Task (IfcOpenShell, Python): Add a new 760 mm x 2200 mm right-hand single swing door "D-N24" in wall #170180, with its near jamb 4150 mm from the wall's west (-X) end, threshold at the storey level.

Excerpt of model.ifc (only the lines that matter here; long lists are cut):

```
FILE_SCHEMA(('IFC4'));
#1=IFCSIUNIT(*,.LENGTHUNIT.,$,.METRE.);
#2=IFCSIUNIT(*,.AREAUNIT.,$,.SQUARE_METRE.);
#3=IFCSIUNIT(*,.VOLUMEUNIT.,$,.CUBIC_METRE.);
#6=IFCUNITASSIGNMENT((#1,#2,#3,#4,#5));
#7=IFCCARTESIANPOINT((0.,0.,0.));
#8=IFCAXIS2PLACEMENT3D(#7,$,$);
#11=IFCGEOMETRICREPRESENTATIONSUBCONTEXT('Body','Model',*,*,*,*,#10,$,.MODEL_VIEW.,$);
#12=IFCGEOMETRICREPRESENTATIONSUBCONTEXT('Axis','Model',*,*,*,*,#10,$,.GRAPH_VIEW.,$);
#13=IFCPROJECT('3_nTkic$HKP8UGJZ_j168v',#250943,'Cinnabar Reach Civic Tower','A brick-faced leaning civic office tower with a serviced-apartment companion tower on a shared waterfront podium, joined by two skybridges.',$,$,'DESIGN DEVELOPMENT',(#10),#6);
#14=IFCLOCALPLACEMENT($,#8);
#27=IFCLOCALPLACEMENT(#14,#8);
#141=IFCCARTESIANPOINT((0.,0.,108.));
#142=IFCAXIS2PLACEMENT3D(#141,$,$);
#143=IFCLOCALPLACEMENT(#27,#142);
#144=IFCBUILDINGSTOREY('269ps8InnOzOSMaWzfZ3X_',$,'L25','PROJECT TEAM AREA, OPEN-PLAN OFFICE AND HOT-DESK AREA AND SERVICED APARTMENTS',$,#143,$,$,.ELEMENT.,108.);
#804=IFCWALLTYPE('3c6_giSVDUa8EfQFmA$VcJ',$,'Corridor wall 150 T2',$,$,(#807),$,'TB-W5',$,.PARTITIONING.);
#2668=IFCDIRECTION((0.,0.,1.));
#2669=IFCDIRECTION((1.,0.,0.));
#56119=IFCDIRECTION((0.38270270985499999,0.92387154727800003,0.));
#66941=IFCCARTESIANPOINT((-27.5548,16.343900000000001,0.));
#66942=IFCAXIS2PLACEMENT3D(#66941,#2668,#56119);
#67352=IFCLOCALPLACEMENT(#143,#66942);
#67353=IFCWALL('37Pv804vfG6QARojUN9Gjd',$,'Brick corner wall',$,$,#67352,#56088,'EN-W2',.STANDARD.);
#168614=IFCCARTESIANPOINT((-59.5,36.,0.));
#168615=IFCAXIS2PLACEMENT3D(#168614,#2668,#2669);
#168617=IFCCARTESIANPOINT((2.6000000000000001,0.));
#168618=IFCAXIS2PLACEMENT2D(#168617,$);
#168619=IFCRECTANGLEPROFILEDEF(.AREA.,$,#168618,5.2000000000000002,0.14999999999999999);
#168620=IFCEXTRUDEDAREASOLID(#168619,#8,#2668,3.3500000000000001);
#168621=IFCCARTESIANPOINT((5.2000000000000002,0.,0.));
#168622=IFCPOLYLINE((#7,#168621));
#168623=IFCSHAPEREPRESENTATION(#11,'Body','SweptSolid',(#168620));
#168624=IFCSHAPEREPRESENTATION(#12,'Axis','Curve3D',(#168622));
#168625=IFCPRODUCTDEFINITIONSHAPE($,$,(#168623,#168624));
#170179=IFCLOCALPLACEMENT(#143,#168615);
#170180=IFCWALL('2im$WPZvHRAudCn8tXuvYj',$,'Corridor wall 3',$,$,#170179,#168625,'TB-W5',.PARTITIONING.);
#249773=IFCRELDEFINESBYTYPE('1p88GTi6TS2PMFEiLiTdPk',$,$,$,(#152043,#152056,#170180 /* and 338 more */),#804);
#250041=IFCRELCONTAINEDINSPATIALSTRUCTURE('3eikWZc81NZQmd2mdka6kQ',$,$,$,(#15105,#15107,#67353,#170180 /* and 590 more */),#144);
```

```python
import numpy as np
import ifcopenshell
import ifcopenshell.api.feature
import ifcopenshell.api.geometry
import ifcopenshell.api.root
import ifcopenshell.api.spatial
import ifcopenshell.geom
import ifcopenshell.util.element
import ifcopenshell.util.placement
import ifcopenshell.util.representation
import ifcopenshell.util.shape
import ifcopenshell.util.unit

model = ifcopenshell.open("model.ifc")
unit_scale = ifcopenshell.util.unit.calculate_unit_scale(model)
settings = ifcopenshell.geom.settings()


def volume(element):
    """Net volume in cubic metres, openings subtracted."""
    shape = ifcopenshell.geom.create_shape(settings, element)
    return ifcopenshell.util.shape.get_volume(shape.geometry)


wall = model.by_guid("2im$WPZvHRAudCn8tXuvYj")
storey = ifcopenshell.util.element.get_container(wall, ifc_class="IfcBuildingStorey")
context = ifcopenshell.util.representation.get_context(model, "Model", "Body", "MODEL_VIEW")
before = volume(wall)

width, height, from_end, sill = 0.76, 2.2, 4.15, 0.0  # metres

# The wall runs along its own X axis, and the end named is its -X end.
wall_shape = ifcopenshell.geom.create_shape(settings, wall)
x, y, z = ifcopenshell.util.shape.get_vertices(wall_shape.geometry).T
start = x.min() + from_end
face, thickness = float(y.min()), float(y.max() - y.min())
wall_matrix = ifcopenshell.util.placement.get_local_placement(wall.ObjectPlacement)
level = ifcopenshell.util.placement.get_local_placement(storey.ObjectPlacement)[2, 3]


def in_wall(x, y):
    """Placement at x, y metres in the wall's axes, at sill height."""
    matrix = wall_matrix.copy()
    matrix[:, 3] = wall_matrix @ np.array([x / unit_scale, y / unit_scale, 0.0, 1.0])
    matrix[2, 3] = level + sill / unit_scale
    return matrix


# Opening: a box that overshoots both wall faces by 50 mm.
opening = ifcopenshell.api.root.create_entity(model, ifc_class="IfcOpeningElement", predefined_type="OPENING")
box = ifcopenshell.api.geometry.add_wall_representation(
    model, context=context, length=width, height=height, thickness=thickness + 0.1
)
ifcopenshell.api.geometry.assign_representation(model, product=opening, representation=box)
ifcopenshell.api.geometry.edit_object_placement(model, product=opening, matrix=in_wall(start, face - 0.05), is_si=False)
ifcopenshell.api.feature.add_feature(model, feature=opening, element=wall)

door = ifcopenshell.api.root.create_entity(model, ifc_class="IfcDoor", name="D-N24", predefined_type="DOOR")
door.OverallWidth, door.OverallHeight = width / unit_scale, height / unit_scale
door.OperationType = "SINGLE_SWING_RIGHT"
body = ifcopenshell.api.geometry.add_door_representation(
    model,
    context=context,
    overall_width=door.OverallWidth,
    overall_height=door.OverallHeight,
    operation_type="SINGLE_SWING_RIGHT",
    lining_properties={"LiningDepth": thickness / unit_scale, "ThresholdDepth": thickness / unit_scale},
)
ifcopenshell.api.geometry.assign_representation(model, product=door, representation=body)
ifcopenshell.api.spatial.assign_container(model, products=[door], relating_structure=storey)
ifcopenshell.api.feature.add_filling(model, opening=opening, element=door)

# The lining spans the wall, so the door starts at the wall face.
ifcopenshell.api.geometry.edit_object_placement(model, product=door, matrix=in_wall(start, face), is_si=False)

after = volume(wall)

print(f"wall volume {before:.3f} -> {after:.3f} m3")

model.write("model_v2.ifc")
```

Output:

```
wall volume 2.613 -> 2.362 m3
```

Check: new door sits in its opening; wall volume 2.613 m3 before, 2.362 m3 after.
